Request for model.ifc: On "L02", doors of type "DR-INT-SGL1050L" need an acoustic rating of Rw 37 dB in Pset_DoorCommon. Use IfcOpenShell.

First a look at what the model holds.

```python
import ifcopenshell
import ifcopenshell.util.element

model = ifcopenshell.open("model.ifc")
print(model.schema)
storey = next(s for s in model.by_type("IfcBuildingStorey") if s.Name == "L02")
doors = [e for e in ifcopenshell.util.element.get_decomposition(storey) if e.is_a("IfcDoor")]
seen = {}
for e in doors:
    element_type = ifcopenshell.util.element.get_type(e)
    key = (element_type.Name if element_type != e and element_type else None, ifcopenshell.util.element.get_pset(e, "Pset_DoorCommon", "AcousticRating"))
    seen[key] = seen.get(key, 0) + 1
for (name, value), count in sorted(seen.items(), key=str):
    print(count, "x", name, "|", value)
```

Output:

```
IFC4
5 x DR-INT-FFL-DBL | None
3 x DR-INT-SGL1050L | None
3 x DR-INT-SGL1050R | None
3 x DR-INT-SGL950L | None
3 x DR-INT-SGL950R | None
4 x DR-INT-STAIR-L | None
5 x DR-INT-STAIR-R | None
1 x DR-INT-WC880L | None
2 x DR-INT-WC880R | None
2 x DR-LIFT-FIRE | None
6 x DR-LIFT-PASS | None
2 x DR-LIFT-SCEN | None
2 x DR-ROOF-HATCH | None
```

```python
import ifcopenshell
import ifcopenshell.api.pset
import ifcopenshell.util.element

model = ifcopenshell.open("model.ifc")

storey = next(s for s in model.by_type("IfcBuildingStorey") if s.Name == "L02")
doors = [e for e in ifcopenshell.util.element.get_decomposition(storey) if e.is_a("IfcDoor")]

count = 0
for e in doors:
    element_type = ifcopenshell.util.element.get_type(e)
    if element_type in (None, e) or element_type.Name != "DR-INT-SGL1050L":
        continue
    # add_pset returns the element's existing set when there is one.
    pset = ifcopenshell.api.pset.add_pset(model, product=e, name="Pset_DoorCommon")
    ifcopenshell.api.pset.edit_pset(model, pset=pset, properties={"AcousticRating": "Rw 37 dB"})
    count += 1

print(count, "doors updated")

model.write("model-out.ifc")
```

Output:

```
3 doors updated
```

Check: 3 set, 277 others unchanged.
